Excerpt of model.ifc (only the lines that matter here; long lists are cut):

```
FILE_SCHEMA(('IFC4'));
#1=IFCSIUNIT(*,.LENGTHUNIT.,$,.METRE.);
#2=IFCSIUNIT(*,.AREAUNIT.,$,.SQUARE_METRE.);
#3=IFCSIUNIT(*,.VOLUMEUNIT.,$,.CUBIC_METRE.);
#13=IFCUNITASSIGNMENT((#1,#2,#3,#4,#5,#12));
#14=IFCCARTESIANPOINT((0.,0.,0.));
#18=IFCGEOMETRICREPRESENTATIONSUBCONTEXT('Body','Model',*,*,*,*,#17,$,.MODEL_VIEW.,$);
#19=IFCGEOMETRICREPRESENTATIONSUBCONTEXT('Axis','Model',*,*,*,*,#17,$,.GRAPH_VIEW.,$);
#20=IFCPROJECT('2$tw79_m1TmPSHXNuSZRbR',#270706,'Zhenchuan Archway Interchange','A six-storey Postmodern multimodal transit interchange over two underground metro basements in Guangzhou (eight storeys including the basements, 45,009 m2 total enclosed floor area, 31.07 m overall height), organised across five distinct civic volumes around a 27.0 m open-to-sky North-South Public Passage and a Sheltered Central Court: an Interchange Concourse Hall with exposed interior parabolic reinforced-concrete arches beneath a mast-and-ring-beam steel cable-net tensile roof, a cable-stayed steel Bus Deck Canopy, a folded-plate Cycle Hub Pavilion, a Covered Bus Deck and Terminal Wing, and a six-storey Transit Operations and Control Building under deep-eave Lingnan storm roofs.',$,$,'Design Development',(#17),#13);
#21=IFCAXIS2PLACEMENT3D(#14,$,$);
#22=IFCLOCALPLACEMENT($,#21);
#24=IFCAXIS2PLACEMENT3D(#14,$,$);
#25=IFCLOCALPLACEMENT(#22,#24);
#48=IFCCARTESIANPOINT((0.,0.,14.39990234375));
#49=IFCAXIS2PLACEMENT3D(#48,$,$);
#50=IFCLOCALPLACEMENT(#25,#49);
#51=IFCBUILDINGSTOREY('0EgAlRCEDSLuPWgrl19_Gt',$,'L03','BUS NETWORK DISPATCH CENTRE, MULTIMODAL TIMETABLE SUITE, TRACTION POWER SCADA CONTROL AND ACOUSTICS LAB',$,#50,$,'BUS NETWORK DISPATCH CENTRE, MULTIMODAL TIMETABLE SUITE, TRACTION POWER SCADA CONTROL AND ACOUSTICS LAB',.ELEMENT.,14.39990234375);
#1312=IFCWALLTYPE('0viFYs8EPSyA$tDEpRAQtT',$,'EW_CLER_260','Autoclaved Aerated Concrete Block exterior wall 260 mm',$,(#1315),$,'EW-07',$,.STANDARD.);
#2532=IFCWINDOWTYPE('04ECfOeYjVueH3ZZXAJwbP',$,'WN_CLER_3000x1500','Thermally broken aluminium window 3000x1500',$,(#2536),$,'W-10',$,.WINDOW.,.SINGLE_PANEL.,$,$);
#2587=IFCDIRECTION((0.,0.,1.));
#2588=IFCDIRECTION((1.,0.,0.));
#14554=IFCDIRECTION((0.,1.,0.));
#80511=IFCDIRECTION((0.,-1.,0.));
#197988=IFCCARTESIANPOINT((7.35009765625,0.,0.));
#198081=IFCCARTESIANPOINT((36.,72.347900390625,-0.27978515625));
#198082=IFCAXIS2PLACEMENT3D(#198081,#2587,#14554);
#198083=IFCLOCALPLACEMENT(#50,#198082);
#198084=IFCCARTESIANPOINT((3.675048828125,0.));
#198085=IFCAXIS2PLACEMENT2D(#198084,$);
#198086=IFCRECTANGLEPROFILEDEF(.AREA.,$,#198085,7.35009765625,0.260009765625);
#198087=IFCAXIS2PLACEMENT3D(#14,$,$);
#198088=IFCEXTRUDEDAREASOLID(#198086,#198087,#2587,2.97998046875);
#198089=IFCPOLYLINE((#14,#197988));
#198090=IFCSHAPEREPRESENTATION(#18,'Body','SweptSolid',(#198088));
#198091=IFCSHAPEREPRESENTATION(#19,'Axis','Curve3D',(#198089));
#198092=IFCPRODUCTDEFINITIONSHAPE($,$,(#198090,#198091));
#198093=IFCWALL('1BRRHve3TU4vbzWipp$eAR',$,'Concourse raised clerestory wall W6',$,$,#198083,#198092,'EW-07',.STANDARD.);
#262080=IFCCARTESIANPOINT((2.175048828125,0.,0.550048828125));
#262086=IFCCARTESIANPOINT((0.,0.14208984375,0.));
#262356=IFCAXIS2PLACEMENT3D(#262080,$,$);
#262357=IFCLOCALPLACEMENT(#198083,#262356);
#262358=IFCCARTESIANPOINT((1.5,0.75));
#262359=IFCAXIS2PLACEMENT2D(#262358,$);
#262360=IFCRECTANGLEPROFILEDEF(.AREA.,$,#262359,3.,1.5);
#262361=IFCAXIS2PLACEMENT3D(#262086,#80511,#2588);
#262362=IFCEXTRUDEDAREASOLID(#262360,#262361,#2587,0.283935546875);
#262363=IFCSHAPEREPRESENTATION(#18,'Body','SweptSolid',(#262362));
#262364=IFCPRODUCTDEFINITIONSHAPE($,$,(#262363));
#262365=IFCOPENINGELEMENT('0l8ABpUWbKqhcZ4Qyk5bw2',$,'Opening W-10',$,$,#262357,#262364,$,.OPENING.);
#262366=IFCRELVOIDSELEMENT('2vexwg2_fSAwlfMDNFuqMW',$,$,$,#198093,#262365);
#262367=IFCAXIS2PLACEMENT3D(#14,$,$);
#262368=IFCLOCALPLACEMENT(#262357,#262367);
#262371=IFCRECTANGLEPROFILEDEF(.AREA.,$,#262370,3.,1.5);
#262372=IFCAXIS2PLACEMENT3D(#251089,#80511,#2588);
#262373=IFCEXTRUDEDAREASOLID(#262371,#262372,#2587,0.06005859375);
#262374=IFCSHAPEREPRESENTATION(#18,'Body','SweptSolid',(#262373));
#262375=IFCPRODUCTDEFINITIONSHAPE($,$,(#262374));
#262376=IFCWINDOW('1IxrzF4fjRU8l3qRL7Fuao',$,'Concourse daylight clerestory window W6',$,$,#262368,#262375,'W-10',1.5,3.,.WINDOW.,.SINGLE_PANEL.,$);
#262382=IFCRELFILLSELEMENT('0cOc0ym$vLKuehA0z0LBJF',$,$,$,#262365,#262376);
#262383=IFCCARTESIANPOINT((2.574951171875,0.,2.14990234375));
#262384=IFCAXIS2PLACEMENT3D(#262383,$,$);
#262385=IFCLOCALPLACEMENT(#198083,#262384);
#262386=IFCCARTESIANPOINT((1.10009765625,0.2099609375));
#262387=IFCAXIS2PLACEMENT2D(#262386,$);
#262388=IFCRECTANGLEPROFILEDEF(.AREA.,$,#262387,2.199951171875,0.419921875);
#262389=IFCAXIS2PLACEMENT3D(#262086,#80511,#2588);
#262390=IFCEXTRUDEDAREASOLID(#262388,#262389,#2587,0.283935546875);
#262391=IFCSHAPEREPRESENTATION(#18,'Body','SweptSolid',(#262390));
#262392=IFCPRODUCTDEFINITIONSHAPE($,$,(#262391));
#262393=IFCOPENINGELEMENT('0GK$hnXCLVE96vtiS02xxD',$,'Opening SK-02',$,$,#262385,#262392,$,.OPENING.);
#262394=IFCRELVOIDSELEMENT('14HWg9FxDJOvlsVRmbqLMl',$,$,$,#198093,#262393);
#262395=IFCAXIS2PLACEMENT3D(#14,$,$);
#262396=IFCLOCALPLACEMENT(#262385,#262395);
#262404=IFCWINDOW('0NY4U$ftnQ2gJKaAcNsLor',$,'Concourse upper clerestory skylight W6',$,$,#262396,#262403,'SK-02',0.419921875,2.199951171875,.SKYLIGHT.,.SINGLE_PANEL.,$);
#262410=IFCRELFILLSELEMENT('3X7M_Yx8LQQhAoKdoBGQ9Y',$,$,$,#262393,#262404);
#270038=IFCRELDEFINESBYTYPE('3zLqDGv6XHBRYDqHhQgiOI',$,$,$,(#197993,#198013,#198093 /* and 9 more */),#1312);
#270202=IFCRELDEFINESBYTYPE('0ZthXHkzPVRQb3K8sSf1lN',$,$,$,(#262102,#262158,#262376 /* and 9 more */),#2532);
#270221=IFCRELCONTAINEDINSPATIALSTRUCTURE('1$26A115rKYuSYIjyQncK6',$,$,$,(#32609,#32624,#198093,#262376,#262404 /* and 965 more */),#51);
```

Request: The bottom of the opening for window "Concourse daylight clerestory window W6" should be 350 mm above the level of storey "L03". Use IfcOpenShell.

```python
import numpy as np
import ifcopenshell
import ifcopenshell.api.geometry
import ifcopenshell.geom
import ifcopenshell.util.element
import ifcopenshell.util.placement
import ifcopenshell.util.shape
import ifcopenshell.util.unit

model = ifcopenshell.open("model.ifc")
unit_scale = ifcopenshell.util.unit.calculate_unit_scale(model)

window = model.by_guid("1IxrzF4fjRU8l3qRL7Fuao")
opening = window.FillsVoids[0].RelatingOpeningElement
storey = ifcopenshell.util.element.get_container(window, ifc_class="IfcBuildingStorey")
level = ifcopenshell.util.placement.get_local_placement(storey.ObjectPlacement)[2, 3]

# The opening's origin need not be at the sill, so measure its lowest point.
shape = ifcopenshell.geom.create_shape(ifcopenshell.geom.settings(), opening)
bottom = ifcopenshell.util.shape.get_shape_bottom_elevation(shape, shape.geometry) / unit_scale
dz = level + 0.35 / unit_scale - bottom

shift = np.array([0.0, 0.0, dz])
# The window is placed relative to its opening, so it follows when the opening moves.
matrix = ifcopenshell.util.placement.get_local_placement(opening.ObjectPlacement)
matrix[:3, 3] += shift
ifcopenshell.api.geometry.edit_object_placement(
    model, product=opening, matrix=matrix, is_si=False, should_transform_children=True
)

print(f"moved by {dz * unit_scale:+.3f} m")

model.write("model_edited.ifc")
```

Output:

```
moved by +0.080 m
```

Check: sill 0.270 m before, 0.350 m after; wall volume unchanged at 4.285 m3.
